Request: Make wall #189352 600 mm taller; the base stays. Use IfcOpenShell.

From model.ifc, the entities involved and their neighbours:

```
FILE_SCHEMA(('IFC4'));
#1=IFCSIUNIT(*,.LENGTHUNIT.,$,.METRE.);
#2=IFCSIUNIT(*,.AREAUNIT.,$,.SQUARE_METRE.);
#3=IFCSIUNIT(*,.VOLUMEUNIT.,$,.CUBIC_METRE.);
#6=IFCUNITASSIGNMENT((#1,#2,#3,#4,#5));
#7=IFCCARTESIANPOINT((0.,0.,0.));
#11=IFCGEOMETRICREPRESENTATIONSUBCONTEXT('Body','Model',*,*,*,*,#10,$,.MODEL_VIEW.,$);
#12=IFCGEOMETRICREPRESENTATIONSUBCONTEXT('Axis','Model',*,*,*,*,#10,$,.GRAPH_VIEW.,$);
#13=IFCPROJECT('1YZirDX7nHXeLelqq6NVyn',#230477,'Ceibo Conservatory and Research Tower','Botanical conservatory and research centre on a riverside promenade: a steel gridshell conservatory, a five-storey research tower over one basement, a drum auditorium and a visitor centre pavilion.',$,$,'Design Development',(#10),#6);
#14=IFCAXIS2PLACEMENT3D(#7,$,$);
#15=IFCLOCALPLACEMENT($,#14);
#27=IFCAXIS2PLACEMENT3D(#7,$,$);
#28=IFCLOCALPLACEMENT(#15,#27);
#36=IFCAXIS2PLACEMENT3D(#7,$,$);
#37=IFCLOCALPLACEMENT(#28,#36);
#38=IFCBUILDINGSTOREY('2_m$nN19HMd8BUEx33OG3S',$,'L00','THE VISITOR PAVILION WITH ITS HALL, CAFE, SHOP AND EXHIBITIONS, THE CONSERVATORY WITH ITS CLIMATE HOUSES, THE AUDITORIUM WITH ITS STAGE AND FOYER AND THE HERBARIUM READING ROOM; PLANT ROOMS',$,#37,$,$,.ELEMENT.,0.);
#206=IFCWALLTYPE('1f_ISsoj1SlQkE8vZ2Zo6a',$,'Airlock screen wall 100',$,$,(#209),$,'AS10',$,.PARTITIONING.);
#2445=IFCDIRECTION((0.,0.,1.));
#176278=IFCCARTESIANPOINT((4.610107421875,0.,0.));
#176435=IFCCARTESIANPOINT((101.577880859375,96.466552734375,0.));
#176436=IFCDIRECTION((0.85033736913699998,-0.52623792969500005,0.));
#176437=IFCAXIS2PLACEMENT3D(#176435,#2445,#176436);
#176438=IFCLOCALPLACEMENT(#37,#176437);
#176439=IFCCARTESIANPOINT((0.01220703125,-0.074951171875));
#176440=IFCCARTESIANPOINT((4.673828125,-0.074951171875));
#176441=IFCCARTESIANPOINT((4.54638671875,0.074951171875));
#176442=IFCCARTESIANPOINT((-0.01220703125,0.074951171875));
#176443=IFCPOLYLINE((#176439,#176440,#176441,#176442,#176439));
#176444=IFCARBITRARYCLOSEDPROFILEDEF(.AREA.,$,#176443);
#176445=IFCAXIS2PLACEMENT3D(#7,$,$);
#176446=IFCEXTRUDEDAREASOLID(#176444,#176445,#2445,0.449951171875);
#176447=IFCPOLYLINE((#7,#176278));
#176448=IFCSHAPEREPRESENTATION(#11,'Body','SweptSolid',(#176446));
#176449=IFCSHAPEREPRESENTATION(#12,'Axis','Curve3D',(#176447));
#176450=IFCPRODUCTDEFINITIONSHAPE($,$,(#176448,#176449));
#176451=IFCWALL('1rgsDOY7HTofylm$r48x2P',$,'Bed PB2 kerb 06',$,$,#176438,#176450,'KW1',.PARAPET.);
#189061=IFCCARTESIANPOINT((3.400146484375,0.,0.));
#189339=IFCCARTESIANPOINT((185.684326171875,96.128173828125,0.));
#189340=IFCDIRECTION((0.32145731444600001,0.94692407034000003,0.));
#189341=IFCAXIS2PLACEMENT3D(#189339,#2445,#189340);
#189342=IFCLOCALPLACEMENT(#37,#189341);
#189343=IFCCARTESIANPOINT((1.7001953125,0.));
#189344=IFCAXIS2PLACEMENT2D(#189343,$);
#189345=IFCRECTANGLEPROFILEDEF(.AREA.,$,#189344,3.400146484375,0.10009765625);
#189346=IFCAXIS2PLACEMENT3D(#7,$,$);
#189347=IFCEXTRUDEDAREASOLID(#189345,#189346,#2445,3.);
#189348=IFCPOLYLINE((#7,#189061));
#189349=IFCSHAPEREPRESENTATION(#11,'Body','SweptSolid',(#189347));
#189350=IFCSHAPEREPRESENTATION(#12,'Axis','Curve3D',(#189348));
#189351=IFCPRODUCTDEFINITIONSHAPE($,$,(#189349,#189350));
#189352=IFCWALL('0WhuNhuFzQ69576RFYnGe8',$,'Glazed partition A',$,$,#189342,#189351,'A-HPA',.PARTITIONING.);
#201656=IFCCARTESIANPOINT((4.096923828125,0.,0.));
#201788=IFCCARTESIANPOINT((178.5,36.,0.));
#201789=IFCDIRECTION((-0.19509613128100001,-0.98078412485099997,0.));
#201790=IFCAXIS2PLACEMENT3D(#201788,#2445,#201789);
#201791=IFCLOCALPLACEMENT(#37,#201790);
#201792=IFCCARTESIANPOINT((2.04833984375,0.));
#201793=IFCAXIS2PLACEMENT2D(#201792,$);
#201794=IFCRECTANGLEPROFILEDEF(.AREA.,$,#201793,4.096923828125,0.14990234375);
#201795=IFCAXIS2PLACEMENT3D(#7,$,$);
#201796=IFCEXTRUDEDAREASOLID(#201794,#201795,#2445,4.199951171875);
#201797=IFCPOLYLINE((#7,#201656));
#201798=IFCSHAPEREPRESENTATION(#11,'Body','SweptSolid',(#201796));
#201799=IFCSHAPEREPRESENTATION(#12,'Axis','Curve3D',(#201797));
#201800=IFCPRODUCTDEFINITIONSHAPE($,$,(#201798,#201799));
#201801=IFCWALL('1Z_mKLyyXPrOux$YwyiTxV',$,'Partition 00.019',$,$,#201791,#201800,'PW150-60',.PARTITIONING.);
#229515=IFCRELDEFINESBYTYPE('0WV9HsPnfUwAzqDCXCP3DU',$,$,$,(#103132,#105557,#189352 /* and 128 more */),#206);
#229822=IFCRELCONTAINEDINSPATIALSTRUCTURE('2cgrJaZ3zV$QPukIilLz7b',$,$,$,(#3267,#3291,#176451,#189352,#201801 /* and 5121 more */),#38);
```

```python
import ifcopenshell
import ifcopenshell.geom
import ifcopenshell.util.representation
import ifcopenshell.util.shape
import ifcopenshell.util.unit

model = ifcopenshell.open("model.ifc")
unit_scale = ifcopenshell.util.unit.calculate_unit_scale(model)
settings = ifcopenshell.geom.settings()


def volume(element):
    """Net volume in cubic metres, openings subtracted."""
    shape = ifcopenshell.geom.create_shape(settings, element)
    return ifcopenshell.util.shape.get_volume(shape.geometry)


wall = model.by_guid("0WhuNhuFzQ69576RFYnGe8")
before = volume(wall)

body = ifcopenshell.util.representation.get_representation(wall, "Model", "Body")
solid = body.Items[0]
old_height = solid.Depth
solid.Depth += 0.6 / unit_scale
after = volume(wall)

print(f"height {old_height:g} -> {solid.Depth:g}, volume {before:.3f} -> {after:.3f} m3")

model.write("model-out.ifc")
```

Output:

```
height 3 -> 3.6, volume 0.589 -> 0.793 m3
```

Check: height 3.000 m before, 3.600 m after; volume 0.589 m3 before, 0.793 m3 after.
